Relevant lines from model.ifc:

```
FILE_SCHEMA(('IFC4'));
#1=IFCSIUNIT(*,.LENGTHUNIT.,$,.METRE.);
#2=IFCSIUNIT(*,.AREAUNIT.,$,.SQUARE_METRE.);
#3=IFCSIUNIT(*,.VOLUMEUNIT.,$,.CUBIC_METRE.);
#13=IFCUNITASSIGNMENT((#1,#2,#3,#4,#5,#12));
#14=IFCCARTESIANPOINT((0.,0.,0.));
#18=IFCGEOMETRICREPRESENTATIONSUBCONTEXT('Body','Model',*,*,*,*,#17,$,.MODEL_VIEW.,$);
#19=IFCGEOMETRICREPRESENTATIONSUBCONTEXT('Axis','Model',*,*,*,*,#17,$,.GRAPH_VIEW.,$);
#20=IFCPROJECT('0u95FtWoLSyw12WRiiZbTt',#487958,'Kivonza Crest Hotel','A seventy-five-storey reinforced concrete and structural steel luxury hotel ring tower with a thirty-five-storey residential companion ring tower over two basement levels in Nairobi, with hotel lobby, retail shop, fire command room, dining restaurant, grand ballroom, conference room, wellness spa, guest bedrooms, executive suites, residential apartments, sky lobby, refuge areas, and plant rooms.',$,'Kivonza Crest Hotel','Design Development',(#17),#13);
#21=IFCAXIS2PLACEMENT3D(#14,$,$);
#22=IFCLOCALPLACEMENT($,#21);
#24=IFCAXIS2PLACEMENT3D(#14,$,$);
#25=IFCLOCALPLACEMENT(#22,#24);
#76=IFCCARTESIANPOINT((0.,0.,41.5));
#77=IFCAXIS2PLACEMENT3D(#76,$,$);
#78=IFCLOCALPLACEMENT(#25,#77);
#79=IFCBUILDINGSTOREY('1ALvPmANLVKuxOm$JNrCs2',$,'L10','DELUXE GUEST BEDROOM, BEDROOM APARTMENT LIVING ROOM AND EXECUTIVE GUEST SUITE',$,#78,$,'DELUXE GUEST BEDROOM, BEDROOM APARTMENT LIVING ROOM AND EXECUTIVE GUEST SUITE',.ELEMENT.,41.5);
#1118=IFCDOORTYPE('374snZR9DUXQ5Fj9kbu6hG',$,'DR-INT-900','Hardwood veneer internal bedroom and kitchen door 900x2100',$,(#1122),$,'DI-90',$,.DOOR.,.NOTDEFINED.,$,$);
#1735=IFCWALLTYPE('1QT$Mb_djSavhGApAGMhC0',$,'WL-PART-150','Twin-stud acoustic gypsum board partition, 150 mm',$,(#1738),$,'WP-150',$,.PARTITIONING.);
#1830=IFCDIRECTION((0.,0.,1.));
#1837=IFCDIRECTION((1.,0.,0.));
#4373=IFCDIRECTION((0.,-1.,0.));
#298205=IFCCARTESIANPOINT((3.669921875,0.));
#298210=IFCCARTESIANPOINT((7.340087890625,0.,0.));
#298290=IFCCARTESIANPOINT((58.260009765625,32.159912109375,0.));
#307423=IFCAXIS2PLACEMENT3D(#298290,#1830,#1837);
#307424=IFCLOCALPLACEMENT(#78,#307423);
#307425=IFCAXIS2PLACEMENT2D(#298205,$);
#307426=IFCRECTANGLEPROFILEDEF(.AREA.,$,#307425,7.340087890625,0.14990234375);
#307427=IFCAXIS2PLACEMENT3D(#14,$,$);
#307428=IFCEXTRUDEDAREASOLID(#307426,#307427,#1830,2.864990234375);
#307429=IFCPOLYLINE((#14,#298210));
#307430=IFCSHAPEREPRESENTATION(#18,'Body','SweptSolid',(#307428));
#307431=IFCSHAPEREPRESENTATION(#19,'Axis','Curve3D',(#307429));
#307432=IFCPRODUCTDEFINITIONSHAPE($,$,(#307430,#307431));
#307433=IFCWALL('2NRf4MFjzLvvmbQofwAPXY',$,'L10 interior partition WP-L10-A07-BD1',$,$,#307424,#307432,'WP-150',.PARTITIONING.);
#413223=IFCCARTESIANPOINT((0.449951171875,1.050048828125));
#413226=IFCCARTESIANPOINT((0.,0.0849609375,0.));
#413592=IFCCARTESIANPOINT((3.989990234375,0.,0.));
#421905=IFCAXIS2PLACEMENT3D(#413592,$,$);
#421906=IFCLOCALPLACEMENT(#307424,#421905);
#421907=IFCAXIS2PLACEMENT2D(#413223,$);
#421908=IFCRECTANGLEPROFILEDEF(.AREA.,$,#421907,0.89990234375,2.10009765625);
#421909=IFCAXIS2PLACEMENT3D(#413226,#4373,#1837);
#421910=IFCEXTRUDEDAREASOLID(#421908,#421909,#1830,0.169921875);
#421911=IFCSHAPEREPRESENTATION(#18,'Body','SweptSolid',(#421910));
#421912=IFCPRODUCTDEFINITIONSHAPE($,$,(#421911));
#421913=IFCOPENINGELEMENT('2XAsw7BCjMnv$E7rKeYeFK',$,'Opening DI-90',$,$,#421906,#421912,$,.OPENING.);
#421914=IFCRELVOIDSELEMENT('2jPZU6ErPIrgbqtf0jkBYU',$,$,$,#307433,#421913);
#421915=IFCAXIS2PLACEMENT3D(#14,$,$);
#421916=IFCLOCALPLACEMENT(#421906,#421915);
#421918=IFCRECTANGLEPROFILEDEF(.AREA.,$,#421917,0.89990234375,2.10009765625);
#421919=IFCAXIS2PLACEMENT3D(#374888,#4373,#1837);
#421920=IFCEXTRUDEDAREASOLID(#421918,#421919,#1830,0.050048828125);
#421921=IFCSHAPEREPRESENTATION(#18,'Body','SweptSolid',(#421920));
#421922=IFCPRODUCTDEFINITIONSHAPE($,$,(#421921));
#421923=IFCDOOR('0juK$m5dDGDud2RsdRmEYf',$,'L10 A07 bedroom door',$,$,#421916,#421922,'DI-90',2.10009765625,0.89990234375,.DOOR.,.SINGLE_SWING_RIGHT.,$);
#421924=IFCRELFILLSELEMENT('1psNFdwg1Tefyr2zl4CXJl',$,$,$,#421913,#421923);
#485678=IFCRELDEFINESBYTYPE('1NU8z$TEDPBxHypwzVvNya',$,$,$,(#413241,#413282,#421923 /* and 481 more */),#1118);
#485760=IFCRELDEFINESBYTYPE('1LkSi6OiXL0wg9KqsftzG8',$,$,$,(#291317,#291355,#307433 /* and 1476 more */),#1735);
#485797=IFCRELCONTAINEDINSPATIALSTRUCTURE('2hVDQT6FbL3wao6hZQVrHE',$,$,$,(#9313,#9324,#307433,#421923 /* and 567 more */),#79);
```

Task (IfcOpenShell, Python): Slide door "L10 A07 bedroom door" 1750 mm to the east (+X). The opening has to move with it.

```python
import ifcopenshell
import ifcopenshell.api.geometry
import ifcopenshell.util.placement
import ifcopenshell.util.unit

model = ifcopenshell.open("model.ifc")
unit_scale = ifcopenshell.util.unit.calculate_unit_scale(model)

door = model.by_guid("0juK$m5dDGDud2RsdRmEYf")
opening = door.FillsVoids[0].RelatingOpeningElement
wall = opening.VoidsElements[0].RelatingBuildingElement

wall_matrix = ifcopenshell.util.placement.get_local_placement(wall.ObjectPlacement)
shift = wall_matrix[:3, 0] * 1.75 / unit_scale
before = ifcopenshell.util.placement.get_local_placement(door.ObjectPlacement)[:3, 3].copy()

# The door is placed relative to its opening, so it follows when the opening moves.
matrix = ifcopenshell.util.placement.get_local_placement(opening.ObjectPlacement)
matrix[:3, 3] += shift
ifcopenshell.api.geometry.edit_object_placement(
    model, product=opening, matrix=matrix, is_si=False, should_transform_children=True
)

after = ifcopenshell.util.placement.get_local_placement(door.ObjectPlacement)[:3, 3]
print("door moved by", (after - before).round(3) + 0.0)

model.write("model-out.ifc")
```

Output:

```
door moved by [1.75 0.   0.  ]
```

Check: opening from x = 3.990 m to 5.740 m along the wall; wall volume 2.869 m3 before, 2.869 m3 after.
